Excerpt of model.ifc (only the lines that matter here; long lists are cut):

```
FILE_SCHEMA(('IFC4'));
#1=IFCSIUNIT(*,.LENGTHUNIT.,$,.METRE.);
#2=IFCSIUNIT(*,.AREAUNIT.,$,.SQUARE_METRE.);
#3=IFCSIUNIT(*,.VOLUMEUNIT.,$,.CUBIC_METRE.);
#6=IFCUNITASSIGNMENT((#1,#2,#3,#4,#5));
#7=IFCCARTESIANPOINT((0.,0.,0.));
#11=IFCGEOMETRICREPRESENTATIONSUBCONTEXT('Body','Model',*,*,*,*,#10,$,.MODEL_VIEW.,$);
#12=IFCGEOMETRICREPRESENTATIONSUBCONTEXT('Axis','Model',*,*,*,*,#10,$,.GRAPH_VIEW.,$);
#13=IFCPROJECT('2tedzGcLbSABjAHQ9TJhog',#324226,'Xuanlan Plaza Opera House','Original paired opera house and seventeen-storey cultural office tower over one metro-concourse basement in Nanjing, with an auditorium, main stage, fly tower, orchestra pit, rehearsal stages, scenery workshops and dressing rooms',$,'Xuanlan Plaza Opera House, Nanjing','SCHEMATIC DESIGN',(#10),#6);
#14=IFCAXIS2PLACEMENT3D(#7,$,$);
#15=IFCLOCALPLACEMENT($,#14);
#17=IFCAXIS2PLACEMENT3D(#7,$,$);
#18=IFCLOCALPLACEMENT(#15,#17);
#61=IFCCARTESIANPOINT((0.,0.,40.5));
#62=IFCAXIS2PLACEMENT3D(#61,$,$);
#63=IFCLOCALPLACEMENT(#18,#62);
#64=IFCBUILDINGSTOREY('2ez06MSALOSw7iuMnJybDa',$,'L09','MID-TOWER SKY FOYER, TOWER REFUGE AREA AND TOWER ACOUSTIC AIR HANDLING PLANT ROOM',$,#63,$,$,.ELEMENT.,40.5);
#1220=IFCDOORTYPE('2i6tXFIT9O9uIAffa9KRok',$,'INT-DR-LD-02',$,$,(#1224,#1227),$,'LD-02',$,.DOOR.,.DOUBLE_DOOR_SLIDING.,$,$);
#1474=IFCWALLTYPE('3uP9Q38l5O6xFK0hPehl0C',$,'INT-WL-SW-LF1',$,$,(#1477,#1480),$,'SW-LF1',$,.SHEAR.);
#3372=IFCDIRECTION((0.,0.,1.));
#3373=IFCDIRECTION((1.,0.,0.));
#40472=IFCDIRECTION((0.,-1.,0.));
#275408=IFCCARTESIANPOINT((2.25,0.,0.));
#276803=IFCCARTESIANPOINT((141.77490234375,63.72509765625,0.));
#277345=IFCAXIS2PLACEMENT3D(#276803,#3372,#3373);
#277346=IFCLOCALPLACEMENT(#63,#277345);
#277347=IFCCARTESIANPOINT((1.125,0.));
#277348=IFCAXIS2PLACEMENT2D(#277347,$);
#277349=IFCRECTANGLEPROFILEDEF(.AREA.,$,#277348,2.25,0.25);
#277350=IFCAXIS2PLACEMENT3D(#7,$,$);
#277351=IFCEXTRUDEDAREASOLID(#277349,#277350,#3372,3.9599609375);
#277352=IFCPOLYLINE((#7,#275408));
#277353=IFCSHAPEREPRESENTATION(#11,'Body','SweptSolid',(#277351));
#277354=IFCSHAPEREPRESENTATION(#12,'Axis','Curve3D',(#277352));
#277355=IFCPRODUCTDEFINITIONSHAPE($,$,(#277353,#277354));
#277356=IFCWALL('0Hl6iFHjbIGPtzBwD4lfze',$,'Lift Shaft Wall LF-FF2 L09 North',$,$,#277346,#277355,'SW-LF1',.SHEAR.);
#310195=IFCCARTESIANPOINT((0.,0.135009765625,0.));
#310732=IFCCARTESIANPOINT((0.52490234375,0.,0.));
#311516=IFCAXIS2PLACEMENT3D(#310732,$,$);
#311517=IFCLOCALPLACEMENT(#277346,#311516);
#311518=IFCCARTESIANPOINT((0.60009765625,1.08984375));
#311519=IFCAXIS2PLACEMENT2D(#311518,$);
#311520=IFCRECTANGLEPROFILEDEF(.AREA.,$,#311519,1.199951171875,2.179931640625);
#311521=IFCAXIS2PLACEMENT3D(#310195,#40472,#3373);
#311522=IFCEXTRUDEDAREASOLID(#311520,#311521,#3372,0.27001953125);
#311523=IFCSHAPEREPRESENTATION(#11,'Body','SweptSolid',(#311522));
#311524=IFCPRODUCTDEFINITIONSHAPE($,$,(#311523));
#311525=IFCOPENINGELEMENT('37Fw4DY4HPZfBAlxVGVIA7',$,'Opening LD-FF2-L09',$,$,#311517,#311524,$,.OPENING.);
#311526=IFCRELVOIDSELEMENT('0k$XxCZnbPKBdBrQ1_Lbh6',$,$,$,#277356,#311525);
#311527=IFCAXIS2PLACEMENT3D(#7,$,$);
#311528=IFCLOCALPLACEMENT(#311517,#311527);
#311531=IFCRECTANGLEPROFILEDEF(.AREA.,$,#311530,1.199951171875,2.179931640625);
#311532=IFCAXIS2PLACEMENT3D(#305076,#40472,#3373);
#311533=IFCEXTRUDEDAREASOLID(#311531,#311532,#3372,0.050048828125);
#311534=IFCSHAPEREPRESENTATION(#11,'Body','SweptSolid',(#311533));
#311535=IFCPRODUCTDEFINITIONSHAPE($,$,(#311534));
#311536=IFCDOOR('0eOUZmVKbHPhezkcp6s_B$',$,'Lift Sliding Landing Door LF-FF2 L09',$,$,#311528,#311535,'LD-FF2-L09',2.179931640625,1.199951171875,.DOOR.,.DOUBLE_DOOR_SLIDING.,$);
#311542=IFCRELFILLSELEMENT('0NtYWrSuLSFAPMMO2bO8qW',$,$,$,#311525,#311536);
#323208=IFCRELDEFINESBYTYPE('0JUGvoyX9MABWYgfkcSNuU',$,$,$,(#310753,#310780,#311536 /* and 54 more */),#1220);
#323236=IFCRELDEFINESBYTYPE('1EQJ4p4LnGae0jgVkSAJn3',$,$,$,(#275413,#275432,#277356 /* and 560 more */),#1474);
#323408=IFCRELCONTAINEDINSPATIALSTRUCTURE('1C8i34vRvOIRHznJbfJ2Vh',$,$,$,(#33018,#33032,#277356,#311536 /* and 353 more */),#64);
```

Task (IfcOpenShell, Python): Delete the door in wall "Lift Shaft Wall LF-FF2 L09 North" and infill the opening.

```python
import ifcopenshell
import ifcopenshell.api.feature
import ifcopenshell.api.root
import ifcopenshell.geom
import ifcopenshell.util.shape

model = ifcopenshell.open("model.ifc")
settings = ifcopenshell.geom.settings()


def volume(element):
    """Net volume in cubic metres, openings subtracted."""
    shape = ifcopenshell.geom.create_shape(settings, element)
    return ifcopenshell.util.shape.get_volume(shape.geometry)


door = model.by_guid("0eOUZmVKbHPhezkcp6s_B$")
opening = door.FillsVoids[0].RelatingOpeningElement
wall = opening.VoidsElements[0].RelatingBuildingElement
before = volume(wall)

ifcopenshell.api.root.remove_product(model, product=door)
ifcopenshell.api.feature.remove_feature(model, feature=opening)

after = volume(wall)

print(f"wall volume {before:.3f} -> {after:.3f} m3")

model.write("model_updated.ifc")
```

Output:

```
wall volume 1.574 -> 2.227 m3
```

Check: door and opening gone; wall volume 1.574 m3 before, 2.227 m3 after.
